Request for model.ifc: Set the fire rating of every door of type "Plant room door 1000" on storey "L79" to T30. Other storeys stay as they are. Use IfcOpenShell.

First a look at what the model holds.

```python
import ifcopenshell
import ifcopenshell.util.element

model = ifcopenshell.open("model.ifc")
print(model.schema)
storey = next(s for s in model.by_type("IfcBuildingStorey") if s.Name == "L79")
doors = [e for e in ifcopenshell.util.element.get_decomposition(storey) if e.is_a("IfcDoor")]
seen = {}
for e in doors:
    element_type = ifcopenshell.util.element.get_type(e)
    key = (element_type.Name if element_type != e and element_type else None, ifcopenshell.util.element.get_pset(e, "Pset_DoorCommon", "FireRating"))
    seen[key] = seen.get(key, 0) + 1
for (name, value), count in sorted(seen.items(), key=str):
    print(count, "x", name, "|", value)
```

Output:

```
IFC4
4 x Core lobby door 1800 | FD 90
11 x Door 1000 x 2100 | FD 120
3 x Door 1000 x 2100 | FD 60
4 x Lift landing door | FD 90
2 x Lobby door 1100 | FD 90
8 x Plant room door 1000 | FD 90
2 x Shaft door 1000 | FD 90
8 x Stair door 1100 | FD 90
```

```python
import ifcopenshell
import ifcopenshell.api.pset
import ifcopenshell.util.element

model = ifcopenshell.open("model.ifc")

storey = next(s for s in model.by_type("IfcBuildingStorey") if s.Name == "L79")
doors = [e for e in ifcopenshell.util.element.get_decomposition(storey) if e.is_a("IfcDoor")]

count = 0
for e in doors:
    element_type = ifcopenshell.util.element.get_type(e)
    if element_type in (None, e) or element_type.Name != "Plant room door 1000":
        continue
    # add_pset returns the element's existing set when there is one.
    pset = ifcopenshell.api.pset.add_pset(model, product=e, name="Pset_DoorCommon")
    ifcopenshell.api.pset.edit_pset(model, pset=pset, properties={"FireRating": "T30"})
    count += 1

print(count, "doors updated")

model.write("model_updated.ifc")
```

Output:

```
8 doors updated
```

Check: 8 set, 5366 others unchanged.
